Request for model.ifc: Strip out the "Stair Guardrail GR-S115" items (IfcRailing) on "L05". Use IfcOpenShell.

First a look at what the model holds.

```python
import ifcopenshell
import ifcopenshell.util.element

model = ifcopenshell.open("model.ifc")
print(model.schema)
storey = next(s for s in model.by_type("IfcBuildingStorey") if s.Name == "L05")
railings = [e for e in ifcopenshell.util.element.get_decomposition(storey) if e.is_a("IfcRailing")]
seen = {}
for e in railings:
    element_type = ifcopenshell.util.element.get_type(e)
    name = element_type.Name if element_type not in (None, e) else None
    seen[name] = seen.get(name, 0) + 1
for name, count in sorted(seen.items(), key=str):
    print(count, "x", name)
```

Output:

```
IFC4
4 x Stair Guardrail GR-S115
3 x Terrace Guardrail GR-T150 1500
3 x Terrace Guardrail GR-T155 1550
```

```python
import ifcopenshell
import ifcopenshell.api.root
import ifcopenshell.util.element

model = ifcopenshell.open("model.ifc")

storey = next(s for s in model.by_type("IfcBuildingStorey") if s.Name == "L05")
railings = [e for e in ifcopenshell.util.element.get_decomposition(storey) if e.is_a("IfcRailing")]
targets = [e for e in railings if (t := ifcopenshell.util.element.get_type(e)) not in (None, e) and t.Name == "Stair Guardrail GR-S115"]

for e in targets:
    ifcopenshell.api.root.remove_product(model, product=e)
print(len(targets), "removed")

model.write("model_edited.ifc")
```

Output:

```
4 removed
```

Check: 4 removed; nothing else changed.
